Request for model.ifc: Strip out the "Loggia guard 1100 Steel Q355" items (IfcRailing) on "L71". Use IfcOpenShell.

First a look at what the model holds.

```python
import ifcopenshell
import ifcopenshell.util.element

model = ifcopenshell.open("model.ifc")
print(model.schema)
storey = next(s for s in model.by_type("IfcBuildingStorey") if s.Name == "L71")
railings = [e for e in ifcopenshell.util.element.get_decomposition(storey) if e.is_a("IfcRailing")]
seen = {}
for e in railings:
    element_type = ifcopenshell.util.element.get_type(e)
    name = element_type.Name if element_type not in (None, e) else None
    seen[name] = seen.get(name, 0) + 1
for name, count in sorted(seen.items(), key=str):
    print(count, "x", name)
```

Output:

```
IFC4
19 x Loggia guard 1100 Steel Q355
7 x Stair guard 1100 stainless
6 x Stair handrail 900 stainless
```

```python
import ifcopenshell
import ifcopenshell.api.root
import ifcopenshell.util.element

model = ifcopenshell.open("model.ifc")

storey = next(s for s in model.by_type("IfcBuildingStorey") if s.Name == "L71")
railings = [e for e in ifcopenshell.util.element.get_decomposition(storey) if e.is_a("IfcRailing")]
targets = [e for e in railings if (t := ifcopenshell.util.element.get_type(e)) not in (None, e) and t.Name == "Loggia guard 1100 Steel Q355"]

for e in targets:
    ifcopenshell.api.root.remove_product(model, product=e)
print(len(targets), "removed")

model.write("model_v2.ifc")
```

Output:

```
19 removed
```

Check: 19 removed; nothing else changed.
